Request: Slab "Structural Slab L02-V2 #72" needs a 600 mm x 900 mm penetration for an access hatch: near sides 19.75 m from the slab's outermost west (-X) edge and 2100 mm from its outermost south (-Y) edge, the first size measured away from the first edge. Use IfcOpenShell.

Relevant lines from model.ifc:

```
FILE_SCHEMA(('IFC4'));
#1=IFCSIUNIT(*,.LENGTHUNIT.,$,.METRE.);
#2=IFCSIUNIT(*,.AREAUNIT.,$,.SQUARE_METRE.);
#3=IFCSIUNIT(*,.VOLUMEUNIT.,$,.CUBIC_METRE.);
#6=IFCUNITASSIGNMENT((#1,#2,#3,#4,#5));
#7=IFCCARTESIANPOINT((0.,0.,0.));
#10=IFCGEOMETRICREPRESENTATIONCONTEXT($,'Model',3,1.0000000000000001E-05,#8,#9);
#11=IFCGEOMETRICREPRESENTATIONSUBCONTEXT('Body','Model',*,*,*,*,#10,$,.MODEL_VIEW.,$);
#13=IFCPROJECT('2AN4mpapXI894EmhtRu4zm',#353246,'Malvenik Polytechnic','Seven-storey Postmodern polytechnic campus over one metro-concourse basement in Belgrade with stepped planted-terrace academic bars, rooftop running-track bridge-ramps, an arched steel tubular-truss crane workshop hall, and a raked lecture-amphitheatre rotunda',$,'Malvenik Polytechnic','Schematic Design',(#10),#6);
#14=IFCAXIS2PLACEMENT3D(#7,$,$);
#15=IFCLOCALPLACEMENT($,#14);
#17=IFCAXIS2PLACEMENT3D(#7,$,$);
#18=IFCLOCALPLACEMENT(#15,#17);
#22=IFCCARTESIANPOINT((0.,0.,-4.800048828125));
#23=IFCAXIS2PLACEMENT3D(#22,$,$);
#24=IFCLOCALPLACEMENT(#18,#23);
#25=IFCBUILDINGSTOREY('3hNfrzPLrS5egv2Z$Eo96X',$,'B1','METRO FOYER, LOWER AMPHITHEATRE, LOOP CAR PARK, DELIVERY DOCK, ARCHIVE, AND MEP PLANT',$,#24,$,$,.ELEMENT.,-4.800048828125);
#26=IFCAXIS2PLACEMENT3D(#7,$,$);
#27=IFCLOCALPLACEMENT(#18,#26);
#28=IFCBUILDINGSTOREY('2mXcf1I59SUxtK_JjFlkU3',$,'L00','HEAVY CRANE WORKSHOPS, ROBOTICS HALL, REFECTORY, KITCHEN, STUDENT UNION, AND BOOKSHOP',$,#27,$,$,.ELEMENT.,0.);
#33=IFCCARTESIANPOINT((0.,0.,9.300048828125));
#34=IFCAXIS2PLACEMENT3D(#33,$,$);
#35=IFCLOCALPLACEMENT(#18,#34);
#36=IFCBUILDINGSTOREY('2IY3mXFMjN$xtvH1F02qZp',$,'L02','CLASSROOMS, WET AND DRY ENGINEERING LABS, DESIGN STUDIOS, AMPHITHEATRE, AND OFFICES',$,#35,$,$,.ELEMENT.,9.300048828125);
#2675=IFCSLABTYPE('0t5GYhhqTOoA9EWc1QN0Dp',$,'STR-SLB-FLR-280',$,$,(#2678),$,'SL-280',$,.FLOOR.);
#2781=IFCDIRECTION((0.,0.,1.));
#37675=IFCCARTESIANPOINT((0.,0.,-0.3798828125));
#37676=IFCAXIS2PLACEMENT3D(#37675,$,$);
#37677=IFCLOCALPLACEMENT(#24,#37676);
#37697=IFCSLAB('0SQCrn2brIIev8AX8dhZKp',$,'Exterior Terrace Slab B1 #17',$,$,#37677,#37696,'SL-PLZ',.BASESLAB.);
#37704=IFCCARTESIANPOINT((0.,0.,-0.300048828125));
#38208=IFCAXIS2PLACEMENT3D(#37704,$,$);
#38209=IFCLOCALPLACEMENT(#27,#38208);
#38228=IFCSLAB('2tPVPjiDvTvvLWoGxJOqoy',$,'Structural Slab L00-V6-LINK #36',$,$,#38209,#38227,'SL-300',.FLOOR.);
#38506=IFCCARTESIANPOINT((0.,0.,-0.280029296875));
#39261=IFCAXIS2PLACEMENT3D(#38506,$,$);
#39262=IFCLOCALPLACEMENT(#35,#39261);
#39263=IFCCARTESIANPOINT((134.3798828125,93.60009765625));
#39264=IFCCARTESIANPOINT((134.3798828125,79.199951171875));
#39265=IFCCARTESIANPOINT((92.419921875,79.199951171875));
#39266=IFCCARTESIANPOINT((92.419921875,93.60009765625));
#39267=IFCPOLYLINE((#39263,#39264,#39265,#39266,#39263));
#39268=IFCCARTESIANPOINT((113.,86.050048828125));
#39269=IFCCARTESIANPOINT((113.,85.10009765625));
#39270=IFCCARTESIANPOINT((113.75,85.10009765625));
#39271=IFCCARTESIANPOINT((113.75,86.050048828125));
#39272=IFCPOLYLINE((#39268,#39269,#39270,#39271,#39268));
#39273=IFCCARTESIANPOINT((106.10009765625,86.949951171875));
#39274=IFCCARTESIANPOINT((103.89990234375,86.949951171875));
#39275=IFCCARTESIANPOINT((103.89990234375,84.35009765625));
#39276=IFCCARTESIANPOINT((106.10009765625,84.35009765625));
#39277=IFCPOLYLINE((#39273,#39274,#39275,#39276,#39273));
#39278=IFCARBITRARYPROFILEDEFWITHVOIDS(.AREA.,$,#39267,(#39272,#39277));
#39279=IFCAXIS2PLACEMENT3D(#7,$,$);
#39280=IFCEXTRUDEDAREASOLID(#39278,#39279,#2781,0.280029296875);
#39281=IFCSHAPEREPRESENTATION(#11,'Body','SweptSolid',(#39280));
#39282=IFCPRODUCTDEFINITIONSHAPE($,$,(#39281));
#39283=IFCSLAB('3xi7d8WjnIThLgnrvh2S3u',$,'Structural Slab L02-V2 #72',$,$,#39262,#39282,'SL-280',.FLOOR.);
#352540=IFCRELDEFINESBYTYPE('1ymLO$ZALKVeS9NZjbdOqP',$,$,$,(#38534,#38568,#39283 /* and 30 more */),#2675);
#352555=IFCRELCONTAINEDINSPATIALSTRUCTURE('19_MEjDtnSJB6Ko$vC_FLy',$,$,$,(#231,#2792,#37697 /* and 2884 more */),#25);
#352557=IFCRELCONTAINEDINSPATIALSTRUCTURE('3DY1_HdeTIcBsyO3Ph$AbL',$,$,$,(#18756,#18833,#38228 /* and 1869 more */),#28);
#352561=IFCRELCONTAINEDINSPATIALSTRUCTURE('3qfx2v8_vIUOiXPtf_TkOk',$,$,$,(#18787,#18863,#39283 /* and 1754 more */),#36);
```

```python
import numpy as np
import ifcopenshell
import ifcopenshell.api.feature
import ifcopenshell.api.geometry
import ifcopenshell.api.root
import ifcopenshell.geom
import ifcopenshell.util.placement
import ifcopenshell.util.representation
import ifcopenshell.util.shape
import ifcopenshell.util.unit

model = ifcopenshell.open("model.ifc")
unit_scale = ifcopenshell.util.unit.calculate_unit_scale(model)
settings = ifcopenshell.geom.settings()


def volume(element):
    """Net volume in cubic metres, openings subtracted."""
    shape = ifcopenshell.geom.create_shape(settings, element)
    return ifcopenshell.util.shape.get_volume(shape.geometry)


slab = model.by_guid("3xi7d8WjnIThLgnrvh2S3u")
before = volume(slab)

# Extent in the slab's own axes, in metres. The edges named are its -X and -Y sides.
slab_shape = ifcopenshell.geom.create_shape(settings, slab)
vertices = ifcopenshell.util.shape.get_vertices(slab_shape.geometry)
x_min, y_min, bottom = vertices.min(axis=0)
top = vertices[:, 2].max()

opening = ifcopenshell.api.root.create_entity(model, ifc_class="IfcOpeningElement", name="Access hatch opening", predefined_type="OPENING")
context = ifcopenshell.util.representation.get_context(model, "Model", "Body", "MODEL_VIEW")
width, depth = 0.6, 0.9
outline = [(0.0, 0.0), (width, 0.0), (width, depth), (0.0, depth), (0.0, 0.0)]
# Overshoot both faces by 50 mm so the cut is clean.
shape = ifcopenshell.api.geometry.add_slab_representation(
    model, context=context, depth=top - bottom + 0.1, polyline=outline
)
ifcopenshell.api.geometry.assign_representation(model, product=opening, representation=shape)

matrix = ifcopenshell.util.placement.get_local_placement(slab.ObjectPlacement)
matrix[:, 3] = matrix @ np.append(np.array([x_min + 19.75, y_min + 2.1, bottom - 0.05]) / unit_scale, 1.0)
ifcopenshell.api.geometry.edit_object_placement(model, product=opening, matrix=matrix, is_si=False)
ifcopenshell.api.feature.add_feature(model, feature=opening, element=slab)

after = volume(slab)

print(f"slab volume {before:.3f} -> {after:.3f} m3")

model.write("model_edited.ifc")
```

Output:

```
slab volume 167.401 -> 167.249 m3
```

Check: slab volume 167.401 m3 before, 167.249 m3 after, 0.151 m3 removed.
